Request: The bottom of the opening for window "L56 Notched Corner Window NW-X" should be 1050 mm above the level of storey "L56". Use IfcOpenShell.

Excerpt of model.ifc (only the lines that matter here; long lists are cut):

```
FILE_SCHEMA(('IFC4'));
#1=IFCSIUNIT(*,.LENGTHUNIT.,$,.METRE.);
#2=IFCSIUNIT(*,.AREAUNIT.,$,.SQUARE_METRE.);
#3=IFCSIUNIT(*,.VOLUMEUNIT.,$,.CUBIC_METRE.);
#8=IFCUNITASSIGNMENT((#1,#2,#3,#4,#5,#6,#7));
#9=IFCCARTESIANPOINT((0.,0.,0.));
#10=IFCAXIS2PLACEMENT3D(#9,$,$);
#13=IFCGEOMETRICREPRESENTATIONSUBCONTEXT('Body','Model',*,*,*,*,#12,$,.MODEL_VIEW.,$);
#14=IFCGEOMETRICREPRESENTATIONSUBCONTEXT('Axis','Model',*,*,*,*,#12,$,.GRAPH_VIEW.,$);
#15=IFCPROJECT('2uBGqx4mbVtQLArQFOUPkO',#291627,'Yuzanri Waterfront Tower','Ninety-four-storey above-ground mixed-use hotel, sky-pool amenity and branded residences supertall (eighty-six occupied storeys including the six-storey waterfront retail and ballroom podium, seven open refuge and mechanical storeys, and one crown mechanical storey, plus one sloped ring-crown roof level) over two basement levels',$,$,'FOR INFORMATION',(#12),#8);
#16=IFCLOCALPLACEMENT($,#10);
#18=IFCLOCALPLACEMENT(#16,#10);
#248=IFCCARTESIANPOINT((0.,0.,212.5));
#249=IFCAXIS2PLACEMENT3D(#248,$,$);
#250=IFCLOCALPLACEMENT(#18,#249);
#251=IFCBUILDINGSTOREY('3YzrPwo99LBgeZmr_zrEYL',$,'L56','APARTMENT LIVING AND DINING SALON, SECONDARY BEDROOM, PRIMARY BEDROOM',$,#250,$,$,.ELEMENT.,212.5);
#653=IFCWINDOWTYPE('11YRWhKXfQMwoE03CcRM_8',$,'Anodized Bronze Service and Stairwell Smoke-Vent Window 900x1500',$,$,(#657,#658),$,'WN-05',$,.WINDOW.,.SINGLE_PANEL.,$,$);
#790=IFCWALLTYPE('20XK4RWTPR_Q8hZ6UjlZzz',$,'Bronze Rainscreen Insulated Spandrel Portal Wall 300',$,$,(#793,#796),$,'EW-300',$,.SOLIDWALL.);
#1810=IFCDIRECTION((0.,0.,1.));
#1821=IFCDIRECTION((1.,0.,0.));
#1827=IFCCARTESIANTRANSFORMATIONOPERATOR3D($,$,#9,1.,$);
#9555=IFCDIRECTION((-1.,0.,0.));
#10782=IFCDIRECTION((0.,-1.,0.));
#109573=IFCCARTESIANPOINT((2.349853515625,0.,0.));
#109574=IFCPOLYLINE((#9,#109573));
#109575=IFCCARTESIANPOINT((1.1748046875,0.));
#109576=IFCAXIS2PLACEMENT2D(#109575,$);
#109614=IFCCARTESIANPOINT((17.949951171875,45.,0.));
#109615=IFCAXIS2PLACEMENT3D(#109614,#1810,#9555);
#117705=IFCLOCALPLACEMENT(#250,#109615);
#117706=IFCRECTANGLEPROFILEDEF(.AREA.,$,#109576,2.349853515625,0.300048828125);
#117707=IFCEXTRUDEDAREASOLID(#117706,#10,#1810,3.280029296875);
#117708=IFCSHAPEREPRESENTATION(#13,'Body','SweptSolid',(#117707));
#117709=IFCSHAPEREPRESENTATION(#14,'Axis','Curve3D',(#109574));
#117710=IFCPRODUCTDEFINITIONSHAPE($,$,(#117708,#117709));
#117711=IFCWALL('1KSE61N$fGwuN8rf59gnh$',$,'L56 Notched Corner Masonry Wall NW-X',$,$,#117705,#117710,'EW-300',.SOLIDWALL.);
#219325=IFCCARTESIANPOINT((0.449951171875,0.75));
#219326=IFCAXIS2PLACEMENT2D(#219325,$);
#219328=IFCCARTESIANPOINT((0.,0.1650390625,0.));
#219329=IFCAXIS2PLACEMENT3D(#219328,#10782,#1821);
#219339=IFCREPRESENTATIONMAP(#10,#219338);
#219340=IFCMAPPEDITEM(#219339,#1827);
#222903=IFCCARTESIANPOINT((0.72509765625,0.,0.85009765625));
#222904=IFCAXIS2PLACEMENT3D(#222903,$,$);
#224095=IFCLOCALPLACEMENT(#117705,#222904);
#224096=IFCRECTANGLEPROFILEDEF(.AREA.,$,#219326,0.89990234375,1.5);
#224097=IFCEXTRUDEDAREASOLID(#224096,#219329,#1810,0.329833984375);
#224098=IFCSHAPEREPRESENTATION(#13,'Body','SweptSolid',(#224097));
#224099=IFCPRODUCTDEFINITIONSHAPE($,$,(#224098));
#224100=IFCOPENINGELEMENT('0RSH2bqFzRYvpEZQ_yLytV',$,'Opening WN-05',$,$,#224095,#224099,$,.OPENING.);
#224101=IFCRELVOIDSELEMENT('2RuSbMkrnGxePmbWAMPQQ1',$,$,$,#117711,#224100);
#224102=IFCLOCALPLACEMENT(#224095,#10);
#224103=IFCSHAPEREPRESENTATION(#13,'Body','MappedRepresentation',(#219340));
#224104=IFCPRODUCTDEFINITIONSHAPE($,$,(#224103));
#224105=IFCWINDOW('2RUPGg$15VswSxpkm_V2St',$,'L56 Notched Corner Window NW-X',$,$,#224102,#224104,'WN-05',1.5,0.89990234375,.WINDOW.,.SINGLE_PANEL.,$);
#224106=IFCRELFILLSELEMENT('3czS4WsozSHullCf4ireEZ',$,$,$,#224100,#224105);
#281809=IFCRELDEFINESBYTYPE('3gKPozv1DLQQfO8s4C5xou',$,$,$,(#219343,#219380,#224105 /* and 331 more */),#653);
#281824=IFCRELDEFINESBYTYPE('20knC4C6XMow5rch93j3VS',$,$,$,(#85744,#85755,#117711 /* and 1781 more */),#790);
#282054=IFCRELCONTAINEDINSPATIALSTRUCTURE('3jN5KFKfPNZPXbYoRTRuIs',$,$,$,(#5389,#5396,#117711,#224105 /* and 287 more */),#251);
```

```python
import numpy as np
import ifcopenshell
import ifcopenshell.api.geometry
import ifcopenshell.geom
import ifcopenshell.util.element
import ifcopenshell.util.placement
import ifcopenshell.util.shape
import ifcopenshell.util.unit

model = ifcopenshell.open("model.ifc")
unit_scale = ifcopenshell.util.unit.calculate_unit_scale(model)

window = model.by_guid("2RUPGg$15VswSxpkm_V2St")
opening = window.FillsVoids[0].RelatingOpeningElement
storey = ifcopenshell.util.element.get_container(window, ifc_class="IfcBuildingStorey")
level = ifcopenshell.util.placement.get_local_placement(storey.ObjectPlacement)[2, 3]

# The opening's origin need not be at the sill, so measure its lowest point.
shape = ifcopenshell.geom.create_shape(ifcopenshell.geom.settings(), opening)
bottom = ifcopenshell.util.shape.get_shape_bottom_elevation(shape, shape.geometry) / unit_scale
dz = level + 1.05 / unit_scale - bottom

shift = np.array([0.0, 0.0, dz])
# The window is placed relative to its opening, so it follows when the opening moves.
matrix = ifcopenshell.util.placement.get_local_placement(opening.ObjectPlacement)
matrix[:3, 3] += shift
ifcopenshell.api.geometry.edit_object_placement(
    model, product=opening, matrix=matrix, is_si=False, should_transform_children=True
)

print(f"moved by {dz * unit_scale:+.3f} m")

model.write("model_rev.ifc")
```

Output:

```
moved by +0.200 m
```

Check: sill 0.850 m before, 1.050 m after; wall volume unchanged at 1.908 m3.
